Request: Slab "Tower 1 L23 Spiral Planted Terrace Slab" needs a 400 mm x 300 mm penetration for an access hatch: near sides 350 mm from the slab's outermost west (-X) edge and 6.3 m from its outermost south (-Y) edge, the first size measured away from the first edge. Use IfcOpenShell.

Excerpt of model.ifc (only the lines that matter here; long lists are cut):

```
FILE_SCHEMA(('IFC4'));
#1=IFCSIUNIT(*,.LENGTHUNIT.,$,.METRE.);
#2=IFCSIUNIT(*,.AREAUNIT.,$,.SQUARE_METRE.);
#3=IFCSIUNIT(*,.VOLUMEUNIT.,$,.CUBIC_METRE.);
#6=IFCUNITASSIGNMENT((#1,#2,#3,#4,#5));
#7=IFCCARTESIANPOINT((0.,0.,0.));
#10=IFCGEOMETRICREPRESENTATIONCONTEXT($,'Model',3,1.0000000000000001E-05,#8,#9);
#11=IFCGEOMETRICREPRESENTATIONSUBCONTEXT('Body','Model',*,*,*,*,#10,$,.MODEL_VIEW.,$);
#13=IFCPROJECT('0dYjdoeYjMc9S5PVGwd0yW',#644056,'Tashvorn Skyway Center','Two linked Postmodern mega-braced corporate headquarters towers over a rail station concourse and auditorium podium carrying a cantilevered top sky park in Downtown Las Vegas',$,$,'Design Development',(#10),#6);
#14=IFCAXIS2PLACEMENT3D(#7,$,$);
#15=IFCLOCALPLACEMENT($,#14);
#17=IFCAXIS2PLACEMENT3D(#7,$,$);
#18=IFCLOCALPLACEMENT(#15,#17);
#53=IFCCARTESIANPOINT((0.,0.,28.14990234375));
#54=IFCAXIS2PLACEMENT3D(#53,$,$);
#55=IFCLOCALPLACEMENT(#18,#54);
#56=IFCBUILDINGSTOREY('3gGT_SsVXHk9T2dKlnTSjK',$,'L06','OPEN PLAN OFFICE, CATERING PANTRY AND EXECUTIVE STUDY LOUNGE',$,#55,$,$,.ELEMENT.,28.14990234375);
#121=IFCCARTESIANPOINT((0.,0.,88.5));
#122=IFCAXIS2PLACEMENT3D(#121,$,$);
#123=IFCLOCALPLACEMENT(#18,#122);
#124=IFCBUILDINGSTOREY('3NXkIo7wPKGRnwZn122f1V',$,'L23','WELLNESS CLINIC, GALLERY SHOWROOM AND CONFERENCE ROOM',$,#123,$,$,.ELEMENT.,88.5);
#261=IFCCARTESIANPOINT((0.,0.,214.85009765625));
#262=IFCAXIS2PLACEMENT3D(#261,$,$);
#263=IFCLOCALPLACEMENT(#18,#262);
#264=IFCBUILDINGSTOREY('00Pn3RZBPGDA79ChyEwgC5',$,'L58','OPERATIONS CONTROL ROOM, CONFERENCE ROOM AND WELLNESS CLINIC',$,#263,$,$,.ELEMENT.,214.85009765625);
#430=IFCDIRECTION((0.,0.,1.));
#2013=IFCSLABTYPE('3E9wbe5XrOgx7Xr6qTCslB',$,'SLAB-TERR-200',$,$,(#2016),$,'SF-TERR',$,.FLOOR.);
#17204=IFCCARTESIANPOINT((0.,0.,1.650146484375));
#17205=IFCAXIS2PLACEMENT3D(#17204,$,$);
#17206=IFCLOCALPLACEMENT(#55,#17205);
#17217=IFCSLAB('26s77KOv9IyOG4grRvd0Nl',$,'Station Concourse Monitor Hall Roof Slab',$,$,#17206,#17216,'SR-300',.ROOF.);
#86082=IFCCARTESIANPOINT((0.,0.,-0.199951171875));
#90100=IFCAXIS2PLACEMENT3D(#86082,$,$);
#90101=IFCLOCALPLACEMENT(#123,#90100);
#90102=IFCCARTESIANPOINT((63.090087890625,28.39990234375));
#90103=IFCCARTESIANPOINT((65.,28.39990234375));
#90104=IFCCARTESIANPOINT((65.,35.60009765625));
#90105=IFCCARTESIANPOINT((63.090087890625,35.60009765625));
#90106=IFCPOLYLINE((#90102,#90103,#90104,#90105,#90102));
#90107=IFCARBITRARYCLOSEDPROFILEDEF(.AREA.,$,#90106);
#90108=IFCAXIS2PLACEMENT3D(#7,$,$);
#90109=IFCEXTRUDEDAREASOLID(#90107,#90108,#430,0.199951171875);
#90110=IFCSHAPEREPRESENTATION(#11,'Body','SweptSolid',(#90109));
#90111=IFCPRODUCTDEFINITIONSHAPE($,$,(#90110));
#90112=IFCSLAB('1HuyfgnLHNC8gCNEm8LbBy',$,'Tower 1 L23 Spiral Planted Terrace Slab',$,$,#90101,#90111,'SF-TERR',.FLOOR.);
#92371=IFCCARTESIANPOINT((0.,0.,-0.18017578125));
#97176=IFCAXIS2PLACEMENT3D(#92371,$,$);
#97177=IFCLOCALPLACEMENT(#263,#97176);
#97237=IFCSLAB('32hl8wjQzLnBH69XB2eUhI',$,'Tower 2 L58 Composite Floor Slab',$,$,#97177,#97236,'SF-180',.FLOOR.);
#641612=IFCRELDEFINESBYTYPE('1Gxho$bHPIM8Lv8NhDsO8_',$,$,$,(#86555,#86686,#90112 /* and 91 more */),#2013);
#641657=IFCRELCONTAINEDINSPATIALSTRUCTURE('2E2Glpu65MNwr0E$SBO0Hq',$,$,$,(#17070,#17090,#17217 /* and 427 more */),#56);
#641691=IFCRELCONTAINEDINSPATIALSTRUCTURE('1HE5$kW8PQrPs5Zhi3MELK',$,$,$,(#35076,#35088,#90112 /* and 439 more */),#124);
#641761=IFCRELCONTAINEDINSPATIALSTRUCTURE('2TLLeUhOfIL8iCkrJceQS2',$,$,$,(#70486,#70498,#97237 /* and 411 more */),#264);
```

```python
import numpy as np
import ifcopenshell
import ifcopenshell.api.feature
import ifcopenshell.api.geometry
import ifcopenshell.api.root
import ifcopenshell.geom
import ifcopenshell.util.placement
import ifcopenshell.util.representation
import ifcopenshell.util.shape
import ifcopenshell.util.unit

model = ifcopenshell.open("model.ifc")
unit_scale = ifcopenshell.util.unit.calculate_unit_scale(model)
settings = ifcopenshell.geom.settings()


def volume(element):
    """Net volume in cubic metres, openings subtracted."""
    shape = ifcopenshell.geom.create_shape(settings, element)
    return ifcopenshell.util.shape.get_volume(shape.geometry)


slab = model.by_guid("1HuyfgnLHNC8gCNEm8LbBy")
before = volume(slab)

# Extent in the slab's own axes, in metres. The edges named are its -X and -Y sides.
slab_shape = ifcopenshell.geom.create_shape(settings, slab)
vertices = ifcopenshell.util.shape.get_vertices(slab_shape.geometry)
x_min, y_min, bottom = vertices.min(axis=0)
top = vertices[:, 2].max()

opening = ifcopenshell.api.root.create_entity(model, ifc_class="IfcOpeningElement", name="Access hatch opening", predefined_type="OPENING")
context = ifcopenshell.util.representation.get_context(model, "Model", "Body", "MODEL_VIEW")
width, depth = 0.4, 0.3
outline = [(0.0, 0.0), (width, 0.0), (width, depth), (0.0, depth), (0.0, 0.0)]
# Overshoot both faces by 50 mm so the cut is clean.
shape = ifcopenshell.api.geometry.add_slab_representation(
    model, context=context, depth=top - bottom + 0.1, polyline=outline
)
ifcopenshell.api.geometry.assign_representation(model, product=opening, representation=shape)

matrix = ifcopenshell.util.placement.get_local_placement(slab.ObjectPlacement)
matrix[:, 3] = matrix @ np.append(np.array([x_min + 0.35, y_min + 6.3, bottom - 0.05]) / unit_scale, 1.0)
ifcopenshell.api.geometry.edit_object_placement(model, product=opening, matrix=matrix, is_si=False)
ifcopenshell.api.feature.add_feature(model, feature=opening, element=slab)

after = volume(slab)

print(f"slab volume {before:.3f} -> {after:.3f} m3")

model.write("model-out.ifc")
```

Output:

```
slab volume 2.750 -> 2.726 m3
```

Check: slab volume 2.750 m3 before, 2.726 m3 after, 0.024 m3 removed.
